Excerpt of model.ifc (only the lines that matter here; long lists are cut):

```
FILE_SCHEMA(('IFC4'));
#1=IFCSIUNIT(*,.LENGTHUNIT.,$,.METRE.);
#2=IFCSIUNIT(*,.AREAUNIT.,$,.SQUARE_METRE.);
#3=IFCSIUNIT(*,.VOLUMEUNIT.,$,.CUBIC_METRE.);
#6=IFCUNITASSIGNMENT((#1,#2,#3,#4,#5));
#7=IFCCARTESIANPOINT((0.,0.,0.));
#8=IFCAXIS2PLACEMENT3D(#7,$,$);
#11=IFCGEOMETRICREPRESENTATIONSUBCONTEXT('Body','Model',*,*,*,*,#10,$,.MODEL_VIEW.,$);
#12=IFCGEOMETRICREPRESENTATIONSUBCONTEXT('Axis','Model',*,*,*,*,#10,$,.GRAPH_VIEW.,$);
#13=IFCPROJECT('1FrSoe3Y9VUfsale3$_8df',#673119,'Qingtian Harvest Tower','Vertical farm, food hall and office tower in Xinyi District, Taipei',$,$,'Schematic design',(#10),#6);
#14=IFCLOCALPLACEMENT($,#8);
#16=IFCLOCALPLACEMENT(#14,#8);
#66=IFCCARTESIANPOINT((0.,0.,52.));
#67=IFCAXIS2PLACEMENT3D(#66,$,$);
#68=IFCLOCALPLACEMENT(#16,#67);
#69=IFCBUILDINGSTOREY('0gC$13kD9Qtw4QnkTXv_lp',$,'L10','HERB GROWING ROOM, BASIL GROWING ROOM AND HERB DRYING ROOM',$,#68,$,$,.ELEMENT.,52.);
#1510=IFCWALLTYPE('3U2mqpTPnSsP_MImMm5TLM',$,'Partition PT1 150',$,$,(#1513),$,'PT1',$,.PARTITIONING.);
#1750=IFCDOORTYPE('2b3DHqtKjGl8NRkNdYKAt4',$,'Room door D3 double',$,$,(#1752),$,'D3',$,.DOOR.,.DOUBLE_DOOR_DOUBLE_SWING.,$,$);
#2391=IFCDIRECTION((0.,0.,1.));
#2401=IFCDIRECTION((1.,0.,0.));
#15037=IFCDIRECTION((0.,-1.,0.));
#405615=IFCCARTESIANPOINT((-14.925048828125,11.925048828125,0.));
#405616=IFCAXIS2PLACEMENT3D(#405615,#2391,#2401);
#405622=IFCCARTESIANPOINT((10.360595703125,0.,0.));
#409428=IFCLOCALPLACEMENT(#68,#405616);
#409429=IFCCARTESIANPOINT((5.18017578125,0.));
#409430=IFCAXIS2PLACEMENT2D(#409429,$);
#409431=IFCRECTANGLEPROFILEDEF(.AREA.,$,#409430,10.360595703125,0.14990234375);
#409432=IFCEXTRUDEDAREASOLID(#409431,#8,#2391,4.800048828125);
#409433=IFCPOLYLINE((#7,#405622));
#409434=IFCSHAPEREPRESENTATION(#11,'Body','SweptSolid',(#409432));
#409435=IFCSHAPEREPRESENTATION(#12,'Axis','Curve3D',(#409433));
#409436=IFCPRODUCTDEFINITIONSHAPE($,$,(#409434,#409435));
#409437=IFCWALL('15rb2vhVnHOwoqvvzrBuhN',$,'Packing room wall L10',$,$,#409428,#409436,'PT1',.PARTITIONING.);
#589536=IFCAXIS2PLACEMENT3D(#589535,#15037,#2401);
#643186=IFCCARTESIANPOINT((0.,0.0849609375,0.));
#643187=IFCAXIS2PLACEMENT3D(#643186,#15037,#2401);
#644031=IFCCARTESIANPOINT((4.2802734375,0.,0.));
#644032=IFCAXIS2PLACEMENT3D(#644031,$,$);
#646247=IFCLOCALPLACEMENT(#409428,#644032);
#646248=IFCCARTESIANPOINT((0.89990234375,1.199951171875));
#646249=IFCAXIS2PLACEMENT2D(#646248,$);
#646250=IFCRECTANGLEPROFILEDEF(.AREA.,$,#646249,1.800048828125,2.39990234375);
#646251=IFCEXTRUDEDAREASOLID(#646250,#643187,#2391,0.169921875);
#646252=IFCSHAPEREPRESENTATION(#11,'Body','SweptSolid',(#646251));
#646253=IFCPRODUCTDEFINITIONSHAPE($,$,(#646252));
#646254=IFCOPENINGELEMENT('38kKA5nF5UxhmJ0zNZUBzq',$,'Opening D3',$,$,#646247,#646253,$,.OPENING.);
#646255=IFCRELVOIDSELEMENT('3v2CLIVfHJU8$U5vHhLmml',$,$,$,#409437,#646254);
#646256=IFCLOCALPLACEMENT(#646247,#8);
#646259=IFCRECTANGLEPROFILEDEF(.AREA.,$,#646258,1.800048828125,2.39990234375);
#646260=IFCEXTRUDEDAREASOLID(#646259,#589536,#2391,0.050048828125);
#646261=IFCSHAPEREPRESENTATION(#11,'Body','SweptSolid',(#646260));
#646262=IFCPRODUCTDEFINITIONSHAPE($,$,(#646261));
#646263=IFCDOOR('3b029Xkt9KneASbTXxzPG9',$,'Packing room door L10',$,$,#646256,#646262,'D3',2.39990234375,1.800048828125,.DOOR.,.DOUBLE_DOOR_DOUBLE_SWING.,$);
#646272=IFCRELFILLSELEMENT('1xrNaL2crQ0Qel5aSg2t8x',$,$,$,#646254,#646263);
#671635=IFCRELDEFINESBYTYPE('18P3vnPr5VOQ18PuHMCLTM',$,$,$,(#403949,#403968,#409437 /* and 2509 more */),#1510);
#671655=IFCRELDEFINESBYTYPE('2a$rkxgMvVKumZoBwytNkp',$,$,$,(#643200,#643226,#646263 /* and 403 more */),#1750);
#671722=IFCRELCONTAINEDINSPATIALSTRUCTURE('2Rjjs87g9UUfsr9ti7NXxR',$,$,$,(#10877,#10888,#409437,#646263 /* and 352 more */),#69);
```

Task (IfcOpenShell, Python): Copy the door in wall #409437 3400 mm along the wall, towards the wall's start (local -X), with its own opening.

```python
import ifcopenshell
import ifcopenshell.api.feature
import ifcopenshell.api.geometry
import ifcopenshell.api.root
import ifcopenshell.geom
import ifcopenshell.util.element
import ifcopenshell.util.placement
import ifcopenshell.util.shape
import ifcopenshell.util.unit

model = ifcopenshell.open("model.ifc")
unit_scale = ifcopenshell.util.unit.calculate_unit_scale(model)
settings = ifcopenshell.geom.settings()


def volume(element):
    """Net volume in cubic metres, openings subtracted."""
    shape = ifcopenshell.geom.create_shape(settings, element)
    return ifcopenshell.util.shape.get_volume(shape.geometry)


door = model.by_guid("3b029Xkt9KneASbTXxzPG9")
opening = door.FillsVoids[0].RelatingOpeningElement
wall = opening.VoidsElements[0].RelatingBuildingElement
before = volume(wall)
shift = ifcopenshell.util.placement.get_local_placement(wall.ObjectPlacement)[:3, 0] * -3.4 / unit_scale

# copy_class copies the void relationship, type, container and properties, but no geometry.
new_opening = ifcopenshell.api.root.copy_class(model, product=opening)
new_opening.Representation = ifcopenshell.util.element.copy_deep(
    model, opening.Representation, exclude=["IfcGeometricRepresentationContext", "IfcRepresentationMap"]
)
new_door = ifcopenshell.api.root.copy_class(model, product=door)
new_door.Representation = ifcopenshell.util.element.copy_deep(
    model, door.Representation, exclude=["IfcGeometricRepresentationContext", "IfcRepresentationMap"]
)
new_door.Tag = None
ifcopenshell.api.feature.add_filling(model, opening=new_opening, element=new_door)

for old, new in ((opening, new_opening), (door, new_door)):
    matrix = ifcopenshell.util.placement.get_local_placement(old.ObjectPlacement)
    matrix[:3, 3] += shift
    ifcopenshell.api.geometry.edit_object_placement(model, product=new, matrix=matrix, is_si=False)

after = volume(wall)

print(f"wall volume {before:.3f} -> {after:.3f} m3")

model.write("model_v2.ifc")
```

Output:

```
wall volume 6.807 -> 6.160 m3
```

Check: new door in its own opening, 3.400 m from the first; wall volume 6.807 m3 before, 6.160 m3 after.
